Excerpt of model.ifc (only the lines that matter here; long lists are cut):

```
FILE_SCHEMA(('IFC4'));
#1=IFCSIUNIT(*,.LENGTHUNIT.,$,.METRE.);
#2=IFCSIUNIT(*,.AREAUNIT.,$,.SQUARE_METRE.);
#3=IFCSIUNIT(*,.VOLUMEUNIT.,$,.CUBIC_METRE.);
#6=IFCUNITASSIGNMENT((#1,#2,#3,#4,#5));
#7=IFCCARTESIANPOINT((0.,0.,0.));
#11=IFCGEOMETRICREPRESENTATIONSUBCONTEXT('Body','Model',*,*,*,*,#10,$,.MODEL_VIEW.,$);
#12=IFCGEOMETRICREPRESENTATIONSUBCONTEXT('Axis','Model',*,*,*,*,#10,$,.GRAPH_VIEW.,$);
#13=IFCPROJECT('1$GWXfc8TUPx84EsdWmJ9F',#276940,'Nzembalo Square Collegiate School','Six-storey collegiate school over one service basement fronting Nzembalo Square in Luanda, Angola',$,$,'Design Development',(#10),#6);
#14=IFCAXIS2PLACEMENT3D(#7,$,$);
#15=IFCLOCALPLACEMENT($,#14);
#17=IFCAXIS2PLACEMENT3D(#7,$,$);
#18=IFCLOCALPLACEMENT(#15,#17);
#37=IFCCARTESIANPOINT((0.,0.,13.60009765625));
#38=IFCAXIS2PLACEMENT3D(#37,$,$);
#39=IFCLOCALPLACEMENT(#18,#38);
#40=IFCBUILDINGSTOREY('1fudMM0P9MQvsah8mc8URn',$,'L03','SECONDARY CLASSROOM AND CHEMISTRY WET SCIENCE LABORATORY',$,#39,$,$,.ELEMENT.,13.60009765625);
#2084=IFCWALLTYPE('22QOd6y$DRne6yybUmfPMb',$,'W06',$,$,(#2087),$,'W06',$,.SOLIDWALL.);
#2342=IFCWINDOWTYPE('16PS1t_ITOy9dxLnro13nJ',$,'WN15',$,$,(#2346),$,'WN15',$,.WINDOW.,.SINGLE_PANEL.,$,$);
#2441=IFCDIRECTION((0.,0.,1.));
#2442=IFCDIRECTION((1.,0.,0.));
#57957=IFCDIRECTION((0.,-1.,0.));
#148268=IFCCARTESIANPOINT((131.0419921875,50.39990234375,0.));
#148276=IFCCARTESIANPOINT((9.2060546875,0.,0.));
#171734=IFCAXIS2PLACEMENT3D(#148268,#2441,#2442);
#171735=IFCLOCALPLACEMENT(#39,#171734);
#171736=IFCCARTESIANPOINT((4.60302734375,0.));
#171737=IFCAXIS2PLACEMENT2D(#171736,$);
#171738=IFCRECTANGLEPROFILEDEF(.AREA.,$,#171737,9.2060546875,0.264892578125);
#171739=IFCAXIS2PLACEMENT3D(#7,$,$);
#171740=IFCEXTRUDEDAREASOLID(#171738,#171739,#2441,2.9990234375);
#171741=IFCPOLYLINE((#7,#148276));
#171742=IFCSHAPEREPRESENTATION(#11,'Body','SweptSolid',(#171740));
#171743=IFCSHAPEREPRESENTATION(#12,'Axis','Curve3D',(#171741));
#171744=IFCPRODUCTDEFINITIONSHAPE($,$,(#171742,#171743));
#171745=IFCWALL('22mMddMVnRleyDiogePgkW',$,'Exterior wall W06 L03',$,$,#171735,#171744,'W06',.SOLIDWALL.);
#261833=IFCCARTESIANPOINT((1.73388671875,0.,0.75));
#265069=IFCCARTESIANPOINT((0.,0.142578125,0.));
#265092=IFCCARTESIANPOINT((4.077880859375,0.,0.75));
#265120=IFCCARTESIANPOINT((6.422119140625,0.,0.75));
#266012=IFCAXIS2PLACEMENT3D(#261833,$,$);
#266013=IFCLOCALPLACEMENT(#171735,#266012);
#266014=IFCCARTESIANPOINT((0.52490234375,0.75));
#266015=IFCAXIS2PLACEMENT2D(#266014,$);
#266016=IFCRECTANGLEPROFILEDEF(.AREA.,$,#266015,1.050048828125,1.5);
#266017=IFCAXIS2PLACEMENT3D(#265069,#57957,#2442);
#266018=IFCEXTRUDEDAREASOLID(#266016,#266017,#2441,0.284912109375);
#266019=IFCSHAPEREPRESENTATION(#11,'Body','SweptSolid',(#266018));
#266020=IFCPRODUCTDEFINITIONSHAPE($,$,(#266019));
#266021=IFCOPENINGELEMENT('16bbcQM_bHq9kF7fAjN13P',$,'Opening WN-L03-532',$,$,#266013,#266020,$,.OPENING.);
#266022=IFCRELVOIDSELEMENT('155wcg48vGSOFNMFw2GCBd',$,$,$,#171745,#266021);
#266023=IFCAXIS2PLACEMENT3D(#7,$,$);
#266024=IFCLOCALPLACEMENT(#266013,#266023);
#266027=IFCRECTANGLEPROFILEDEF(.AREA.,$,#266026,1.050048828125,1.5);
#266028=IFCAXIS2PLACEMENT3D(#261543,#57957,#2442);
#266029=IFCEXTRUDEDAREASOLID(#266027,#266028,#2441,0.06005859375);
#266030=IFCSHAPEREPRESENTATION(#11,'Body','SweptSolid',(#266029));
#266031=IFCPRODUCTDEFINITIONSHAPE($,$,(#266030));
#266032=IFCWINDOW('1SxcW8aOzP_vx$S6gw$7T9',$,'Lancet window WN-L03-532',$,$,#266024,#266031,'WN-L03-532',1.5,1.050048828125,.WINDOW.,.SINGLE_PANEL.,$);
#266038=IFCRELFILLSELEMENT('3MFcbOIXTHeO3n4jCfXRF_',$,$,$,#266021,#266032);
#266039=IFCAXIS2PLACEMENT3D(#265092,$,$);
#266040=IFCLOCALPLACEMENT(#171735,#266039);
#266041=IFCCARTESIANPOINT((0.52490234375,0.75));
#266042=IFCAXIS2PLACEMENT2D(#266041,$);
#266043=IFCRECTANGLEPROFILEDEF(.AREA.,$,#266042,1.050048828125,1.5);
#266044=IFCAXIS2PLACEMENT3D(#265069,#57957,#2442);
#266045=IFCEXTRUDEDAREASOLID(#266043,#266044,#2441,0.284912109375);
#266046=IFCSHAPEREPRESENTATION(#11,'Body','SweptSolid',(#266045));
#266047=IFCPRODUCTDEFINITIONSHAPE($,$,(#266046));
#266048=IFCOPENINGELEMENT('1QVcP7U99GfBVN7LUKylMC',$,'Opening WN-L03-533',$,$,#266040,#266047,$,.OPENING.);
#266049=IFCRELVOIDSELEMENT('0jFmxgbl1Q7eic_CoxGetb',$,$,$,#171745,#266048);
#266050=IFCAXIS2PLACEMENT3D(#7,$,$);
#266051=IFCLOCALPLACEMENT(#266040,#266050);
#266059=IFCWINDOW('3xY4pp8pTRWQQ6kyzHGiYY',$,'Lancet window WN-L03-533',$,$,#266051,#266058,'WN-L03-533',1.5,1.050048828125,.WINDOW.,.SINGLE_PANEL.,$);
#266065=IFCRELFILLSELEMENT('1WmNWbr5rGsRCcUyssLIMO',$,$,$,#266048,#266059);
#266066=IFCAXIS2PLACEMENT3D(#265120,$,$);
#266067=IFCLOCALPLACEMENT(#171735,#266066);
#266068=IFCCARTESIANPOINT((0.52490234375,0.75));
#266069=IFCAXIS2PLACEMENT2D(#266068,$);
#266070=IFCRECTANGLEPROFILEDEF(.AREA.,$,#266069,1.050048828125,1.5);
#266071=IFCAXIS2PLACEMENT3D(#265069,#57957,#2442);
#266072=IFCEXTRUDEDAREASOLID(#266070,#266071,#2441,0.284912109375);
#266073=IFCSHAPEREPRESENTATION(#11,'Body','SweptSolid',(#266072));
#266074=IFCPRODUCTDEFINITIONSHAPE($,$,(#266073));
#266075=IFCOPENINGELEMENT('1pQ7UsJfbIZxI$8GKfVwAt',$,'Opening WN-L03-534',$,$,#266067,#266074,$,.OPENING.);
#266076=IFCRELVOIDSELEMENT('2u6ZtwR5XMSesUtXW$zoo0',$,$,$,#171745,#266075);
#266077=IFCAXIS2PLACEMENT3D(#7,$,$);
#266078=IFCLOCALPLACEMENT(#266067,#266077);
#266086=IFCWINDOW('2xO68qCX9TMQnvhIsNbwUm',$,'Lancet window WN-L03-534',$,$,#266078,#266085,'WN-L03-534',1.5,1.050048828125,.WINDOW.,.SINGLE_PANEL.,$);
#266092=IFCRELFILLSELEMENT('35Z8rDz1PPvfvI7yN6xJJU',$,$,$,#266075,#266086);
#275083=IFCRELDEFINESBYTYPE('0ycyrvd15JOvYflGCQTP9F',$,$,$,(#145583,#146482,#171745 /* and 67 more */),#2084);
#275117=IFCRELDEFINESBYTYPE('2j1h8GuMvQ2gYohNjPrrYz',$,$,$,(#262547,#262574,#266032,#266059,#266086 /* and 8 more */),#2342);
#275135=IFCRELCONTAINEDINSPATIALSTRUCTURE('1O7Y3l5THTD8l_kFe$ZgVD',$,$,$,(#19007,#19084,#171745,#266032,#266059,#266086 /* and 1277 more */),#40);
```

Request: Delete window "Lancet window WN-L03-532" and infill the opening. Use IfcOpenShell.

```python
import ifcopenshell
import ifcopenshell.api.feature
import ifcopenshell.api.root
import ifcopenshell.geom
import ifcopenshell.util.shape

model = ifcopenshell.open("model.ifc")
settings = ifcopenshell.geom.settings()


def volume(element):
    """Net volume in cubic metres, openings subtracted."""
    shape = ifcopenshell.geom.create_shape(settings, element)
    return ifcopenshell.util.shape.get_volume(shape.geometry)


window = model.by_guid("1SxcW8aOzP_vx$S6gw$7T9")
opening = window.FillsVoids[0].RelatingOpeningElement
wall = opening.VoidsElements[0].RelatingBuildingElement
before = volume(wall)

ifcopenshell.api.root.remove_product(model, product=window)
ifcopenshell.api.feature.remove_feature(model, feature=opening)

after = volume(wall)

print(f"wall volume {before:.3f} -> {after:.3f} m3")

model.write("model-out.ifc")
```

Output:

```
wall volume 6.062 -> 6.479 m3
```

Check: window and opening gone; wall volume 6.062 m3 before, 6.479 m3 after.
